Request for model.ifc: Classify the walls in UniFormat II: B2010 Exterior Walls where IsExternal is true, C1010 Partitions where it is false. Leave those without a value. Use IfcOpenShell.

First a look at what the model holds.

```python
import ifcopenshell
import ifcopenshell.util.element

model = ifcopenshell.open("model.ifc")
print(model.schema)
print("classifications:", [c.Name for c in model.by_type("IfcClassification")])
values = [ifcopenshell.util.element.get_pset(e, "Pset_WallCommon", "IsExternal") for e in model.by_type("IfcWall")]
for value in (True, False, None):
    print("IsExternal", value, values.count(value))
```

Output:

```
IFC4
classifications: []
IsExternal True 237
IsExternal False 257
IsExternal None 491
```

```python
import ifcopenshell
import ifcopenshell.api.classification
import ifcopenshell.util.element

model = ifcopenshell.open("model.ifc")

system = ifcopenshell.api.classification.add_classification(model, classification="UniFormat II")

walls = model.by_type("IfcWall")
external = {e: ifcopenshell.util.element.get_pset(e, "Pset_WallCommon", "IsExternal") for e in walls}
for flag, code, name in ((True, "B2010", "Exterior Walls"), (False, "C1010", "Partitions")):
    products = [e for e in walls if external[e] is flag]
    ifcopenshell.api.classification.add_reference(
        model, products=products, classification=system, identification=code, name=name
    )
    print(code, len(products))

model.write("model_updated.ifc")
```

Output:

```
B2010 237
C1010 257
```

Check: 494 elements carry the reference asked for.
